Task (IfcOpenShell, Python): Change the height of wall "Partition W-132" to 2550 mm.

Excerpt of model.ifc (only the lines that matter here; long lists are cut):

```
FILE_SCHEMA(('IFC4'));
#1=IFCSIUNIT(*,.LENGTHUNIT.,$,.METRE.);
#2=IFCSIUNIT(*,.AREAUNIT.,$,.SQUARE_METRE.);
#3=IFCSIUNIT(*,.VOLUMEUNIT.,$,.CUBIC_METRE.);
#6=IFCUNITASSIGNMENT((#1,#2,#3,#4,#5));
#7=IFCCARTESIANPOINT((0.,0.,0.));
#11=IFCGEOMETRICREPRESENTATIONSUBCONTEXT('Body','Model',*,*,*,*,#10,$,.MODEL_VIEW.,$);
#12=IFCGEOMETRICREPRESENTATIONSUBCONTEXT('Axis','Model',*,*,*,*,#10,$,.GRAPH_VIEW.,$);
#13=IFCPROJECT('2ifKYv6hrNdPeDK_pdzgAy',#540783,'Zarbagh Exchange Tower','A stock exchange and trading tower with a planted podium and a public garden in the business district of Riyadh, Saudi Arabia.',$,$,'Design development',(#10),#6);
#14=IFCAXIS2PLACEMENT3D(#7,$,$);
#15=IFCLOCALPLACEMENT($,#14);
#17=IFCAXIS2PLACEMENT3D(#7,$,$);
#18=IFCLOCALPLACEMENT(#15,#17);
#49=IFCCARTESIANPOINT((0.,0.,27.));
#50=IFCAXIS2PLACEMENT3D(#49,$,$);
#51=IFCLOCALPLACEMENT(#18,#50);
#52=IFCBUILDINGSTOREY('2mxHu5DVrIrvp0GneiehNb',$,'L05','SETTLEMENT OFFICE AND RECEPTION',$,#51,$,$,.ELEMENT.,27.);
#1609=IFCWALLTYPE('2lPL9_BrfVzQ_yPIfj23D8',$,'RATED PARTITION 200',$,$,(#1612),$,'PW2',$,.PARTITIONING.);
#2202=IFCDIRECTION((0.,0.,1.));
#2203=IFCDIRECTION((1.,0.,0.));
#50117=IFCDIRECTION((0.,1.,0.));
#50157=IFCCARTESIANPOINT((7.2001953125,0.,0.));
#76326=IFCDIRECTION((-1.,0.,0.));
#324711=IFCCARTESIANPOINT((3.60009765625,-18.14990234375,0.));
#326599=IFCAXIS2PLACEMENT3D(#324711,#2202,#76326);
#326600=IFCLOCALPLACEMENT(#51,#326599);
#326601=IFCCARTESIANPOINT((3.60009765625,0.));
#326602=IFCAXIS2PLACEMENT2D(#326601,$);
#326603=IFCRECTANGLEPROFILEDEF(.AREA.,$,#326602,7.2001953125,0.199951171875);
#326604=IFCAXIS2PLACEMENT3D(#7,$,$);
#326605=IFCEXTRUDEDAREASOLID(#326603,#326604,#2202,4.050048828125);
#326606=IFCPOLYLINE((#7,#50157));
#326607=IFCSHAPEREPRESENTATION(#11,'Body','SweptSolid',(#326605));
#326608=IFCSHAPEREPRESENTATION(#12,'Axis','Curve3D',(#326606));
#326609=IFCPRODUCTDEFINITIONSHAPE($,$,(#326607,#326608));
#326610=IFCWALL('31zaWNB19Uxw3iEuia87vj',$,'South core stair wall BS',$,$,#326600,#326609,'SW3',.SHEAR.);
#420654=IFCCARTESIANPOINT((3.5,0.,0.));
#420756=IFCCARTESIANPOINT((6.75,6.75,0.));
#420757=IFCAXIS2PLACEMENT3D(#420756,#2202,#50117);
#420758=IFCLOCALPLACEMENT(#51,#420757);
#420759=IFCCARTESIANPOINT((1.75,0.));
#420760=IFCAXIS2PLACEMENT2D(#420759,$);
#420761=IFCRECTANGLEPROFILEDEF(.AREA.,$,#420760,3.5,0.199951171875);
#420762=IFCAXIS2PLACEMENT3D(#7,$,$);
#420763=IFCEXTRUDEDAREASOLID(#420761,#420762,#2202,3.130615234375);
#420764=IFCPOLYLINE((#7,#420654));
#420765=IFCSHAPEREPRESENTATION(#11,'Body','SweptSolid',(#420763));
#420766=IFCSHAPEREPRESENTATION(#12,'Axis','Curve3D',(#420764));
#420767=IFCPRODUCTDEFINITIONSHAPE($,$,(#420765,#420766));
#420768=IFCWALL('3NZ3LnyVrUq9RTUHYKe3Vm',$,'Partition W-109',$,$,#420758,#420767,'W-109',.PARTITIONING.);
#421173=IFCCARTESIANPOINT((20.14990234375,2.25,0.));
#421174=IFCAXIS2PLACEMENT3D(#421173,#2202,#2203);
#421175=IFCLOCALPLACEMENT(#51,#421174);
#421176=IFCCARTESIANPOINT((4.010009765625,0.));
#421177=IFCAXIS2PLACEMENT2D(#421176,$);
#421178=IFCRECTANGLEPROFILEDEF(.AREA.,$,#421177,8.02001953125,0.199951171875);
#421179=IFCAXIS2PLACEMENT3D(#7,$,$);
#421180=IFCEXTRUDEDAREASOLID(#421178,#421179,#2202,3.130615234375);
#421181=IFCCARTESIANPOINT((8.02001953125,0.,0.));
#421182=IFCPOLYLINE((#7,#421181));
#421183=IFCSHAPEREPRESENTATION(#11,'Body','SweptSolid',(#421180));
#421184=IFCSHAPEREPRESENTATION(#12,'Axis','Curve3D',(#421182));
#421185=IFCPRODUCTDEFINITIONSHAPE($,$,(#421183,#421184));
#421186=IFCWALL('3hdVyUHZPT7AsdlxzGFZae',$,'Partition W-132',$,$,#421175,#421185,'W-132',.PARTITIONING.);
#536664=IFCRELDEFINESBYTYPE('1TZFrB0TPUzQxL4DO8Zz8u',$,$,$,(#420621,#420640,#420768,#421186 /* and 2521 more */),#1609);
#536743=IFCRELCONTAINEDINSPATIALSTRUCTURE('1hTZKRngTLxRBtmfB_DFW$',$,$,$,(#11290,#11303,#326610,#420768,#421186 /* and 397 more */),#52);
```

```python
import ifcopenshell
import ifcopenshell.geom
import ifcopenshell.util.representation
import ifcopenshell.util.shape

model = ifcopenshell.open("model.ifc")
settings = ifcopenshell.geom.settings()


def volume(element):
    """Net volume in cubic metres, openings subtracted."""
    shape = ifcopenshell.geom.create_shape(settings, element)
    return ifcopenshell.util.shape.get_volume(shape.geometry)


wall = model.by_id(421186)
before = volume(wall)

body = ifcopenshell.util.representation.get_representation(wall, "Model", "Body")
solid = body.Items[0]
old_height = solid.Depth
solid.Depth = 2.55
after = volume(wall)

print(f"height {old_height:g} -> {solid.Depth:g}, volume {before:.3f} -> {after:.3f} m3")

model.write("model_v2.ifc")
```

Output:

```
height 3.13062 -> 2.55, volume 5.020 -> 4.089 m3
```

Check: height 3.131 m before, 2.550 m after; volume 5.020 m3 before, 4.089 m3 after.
